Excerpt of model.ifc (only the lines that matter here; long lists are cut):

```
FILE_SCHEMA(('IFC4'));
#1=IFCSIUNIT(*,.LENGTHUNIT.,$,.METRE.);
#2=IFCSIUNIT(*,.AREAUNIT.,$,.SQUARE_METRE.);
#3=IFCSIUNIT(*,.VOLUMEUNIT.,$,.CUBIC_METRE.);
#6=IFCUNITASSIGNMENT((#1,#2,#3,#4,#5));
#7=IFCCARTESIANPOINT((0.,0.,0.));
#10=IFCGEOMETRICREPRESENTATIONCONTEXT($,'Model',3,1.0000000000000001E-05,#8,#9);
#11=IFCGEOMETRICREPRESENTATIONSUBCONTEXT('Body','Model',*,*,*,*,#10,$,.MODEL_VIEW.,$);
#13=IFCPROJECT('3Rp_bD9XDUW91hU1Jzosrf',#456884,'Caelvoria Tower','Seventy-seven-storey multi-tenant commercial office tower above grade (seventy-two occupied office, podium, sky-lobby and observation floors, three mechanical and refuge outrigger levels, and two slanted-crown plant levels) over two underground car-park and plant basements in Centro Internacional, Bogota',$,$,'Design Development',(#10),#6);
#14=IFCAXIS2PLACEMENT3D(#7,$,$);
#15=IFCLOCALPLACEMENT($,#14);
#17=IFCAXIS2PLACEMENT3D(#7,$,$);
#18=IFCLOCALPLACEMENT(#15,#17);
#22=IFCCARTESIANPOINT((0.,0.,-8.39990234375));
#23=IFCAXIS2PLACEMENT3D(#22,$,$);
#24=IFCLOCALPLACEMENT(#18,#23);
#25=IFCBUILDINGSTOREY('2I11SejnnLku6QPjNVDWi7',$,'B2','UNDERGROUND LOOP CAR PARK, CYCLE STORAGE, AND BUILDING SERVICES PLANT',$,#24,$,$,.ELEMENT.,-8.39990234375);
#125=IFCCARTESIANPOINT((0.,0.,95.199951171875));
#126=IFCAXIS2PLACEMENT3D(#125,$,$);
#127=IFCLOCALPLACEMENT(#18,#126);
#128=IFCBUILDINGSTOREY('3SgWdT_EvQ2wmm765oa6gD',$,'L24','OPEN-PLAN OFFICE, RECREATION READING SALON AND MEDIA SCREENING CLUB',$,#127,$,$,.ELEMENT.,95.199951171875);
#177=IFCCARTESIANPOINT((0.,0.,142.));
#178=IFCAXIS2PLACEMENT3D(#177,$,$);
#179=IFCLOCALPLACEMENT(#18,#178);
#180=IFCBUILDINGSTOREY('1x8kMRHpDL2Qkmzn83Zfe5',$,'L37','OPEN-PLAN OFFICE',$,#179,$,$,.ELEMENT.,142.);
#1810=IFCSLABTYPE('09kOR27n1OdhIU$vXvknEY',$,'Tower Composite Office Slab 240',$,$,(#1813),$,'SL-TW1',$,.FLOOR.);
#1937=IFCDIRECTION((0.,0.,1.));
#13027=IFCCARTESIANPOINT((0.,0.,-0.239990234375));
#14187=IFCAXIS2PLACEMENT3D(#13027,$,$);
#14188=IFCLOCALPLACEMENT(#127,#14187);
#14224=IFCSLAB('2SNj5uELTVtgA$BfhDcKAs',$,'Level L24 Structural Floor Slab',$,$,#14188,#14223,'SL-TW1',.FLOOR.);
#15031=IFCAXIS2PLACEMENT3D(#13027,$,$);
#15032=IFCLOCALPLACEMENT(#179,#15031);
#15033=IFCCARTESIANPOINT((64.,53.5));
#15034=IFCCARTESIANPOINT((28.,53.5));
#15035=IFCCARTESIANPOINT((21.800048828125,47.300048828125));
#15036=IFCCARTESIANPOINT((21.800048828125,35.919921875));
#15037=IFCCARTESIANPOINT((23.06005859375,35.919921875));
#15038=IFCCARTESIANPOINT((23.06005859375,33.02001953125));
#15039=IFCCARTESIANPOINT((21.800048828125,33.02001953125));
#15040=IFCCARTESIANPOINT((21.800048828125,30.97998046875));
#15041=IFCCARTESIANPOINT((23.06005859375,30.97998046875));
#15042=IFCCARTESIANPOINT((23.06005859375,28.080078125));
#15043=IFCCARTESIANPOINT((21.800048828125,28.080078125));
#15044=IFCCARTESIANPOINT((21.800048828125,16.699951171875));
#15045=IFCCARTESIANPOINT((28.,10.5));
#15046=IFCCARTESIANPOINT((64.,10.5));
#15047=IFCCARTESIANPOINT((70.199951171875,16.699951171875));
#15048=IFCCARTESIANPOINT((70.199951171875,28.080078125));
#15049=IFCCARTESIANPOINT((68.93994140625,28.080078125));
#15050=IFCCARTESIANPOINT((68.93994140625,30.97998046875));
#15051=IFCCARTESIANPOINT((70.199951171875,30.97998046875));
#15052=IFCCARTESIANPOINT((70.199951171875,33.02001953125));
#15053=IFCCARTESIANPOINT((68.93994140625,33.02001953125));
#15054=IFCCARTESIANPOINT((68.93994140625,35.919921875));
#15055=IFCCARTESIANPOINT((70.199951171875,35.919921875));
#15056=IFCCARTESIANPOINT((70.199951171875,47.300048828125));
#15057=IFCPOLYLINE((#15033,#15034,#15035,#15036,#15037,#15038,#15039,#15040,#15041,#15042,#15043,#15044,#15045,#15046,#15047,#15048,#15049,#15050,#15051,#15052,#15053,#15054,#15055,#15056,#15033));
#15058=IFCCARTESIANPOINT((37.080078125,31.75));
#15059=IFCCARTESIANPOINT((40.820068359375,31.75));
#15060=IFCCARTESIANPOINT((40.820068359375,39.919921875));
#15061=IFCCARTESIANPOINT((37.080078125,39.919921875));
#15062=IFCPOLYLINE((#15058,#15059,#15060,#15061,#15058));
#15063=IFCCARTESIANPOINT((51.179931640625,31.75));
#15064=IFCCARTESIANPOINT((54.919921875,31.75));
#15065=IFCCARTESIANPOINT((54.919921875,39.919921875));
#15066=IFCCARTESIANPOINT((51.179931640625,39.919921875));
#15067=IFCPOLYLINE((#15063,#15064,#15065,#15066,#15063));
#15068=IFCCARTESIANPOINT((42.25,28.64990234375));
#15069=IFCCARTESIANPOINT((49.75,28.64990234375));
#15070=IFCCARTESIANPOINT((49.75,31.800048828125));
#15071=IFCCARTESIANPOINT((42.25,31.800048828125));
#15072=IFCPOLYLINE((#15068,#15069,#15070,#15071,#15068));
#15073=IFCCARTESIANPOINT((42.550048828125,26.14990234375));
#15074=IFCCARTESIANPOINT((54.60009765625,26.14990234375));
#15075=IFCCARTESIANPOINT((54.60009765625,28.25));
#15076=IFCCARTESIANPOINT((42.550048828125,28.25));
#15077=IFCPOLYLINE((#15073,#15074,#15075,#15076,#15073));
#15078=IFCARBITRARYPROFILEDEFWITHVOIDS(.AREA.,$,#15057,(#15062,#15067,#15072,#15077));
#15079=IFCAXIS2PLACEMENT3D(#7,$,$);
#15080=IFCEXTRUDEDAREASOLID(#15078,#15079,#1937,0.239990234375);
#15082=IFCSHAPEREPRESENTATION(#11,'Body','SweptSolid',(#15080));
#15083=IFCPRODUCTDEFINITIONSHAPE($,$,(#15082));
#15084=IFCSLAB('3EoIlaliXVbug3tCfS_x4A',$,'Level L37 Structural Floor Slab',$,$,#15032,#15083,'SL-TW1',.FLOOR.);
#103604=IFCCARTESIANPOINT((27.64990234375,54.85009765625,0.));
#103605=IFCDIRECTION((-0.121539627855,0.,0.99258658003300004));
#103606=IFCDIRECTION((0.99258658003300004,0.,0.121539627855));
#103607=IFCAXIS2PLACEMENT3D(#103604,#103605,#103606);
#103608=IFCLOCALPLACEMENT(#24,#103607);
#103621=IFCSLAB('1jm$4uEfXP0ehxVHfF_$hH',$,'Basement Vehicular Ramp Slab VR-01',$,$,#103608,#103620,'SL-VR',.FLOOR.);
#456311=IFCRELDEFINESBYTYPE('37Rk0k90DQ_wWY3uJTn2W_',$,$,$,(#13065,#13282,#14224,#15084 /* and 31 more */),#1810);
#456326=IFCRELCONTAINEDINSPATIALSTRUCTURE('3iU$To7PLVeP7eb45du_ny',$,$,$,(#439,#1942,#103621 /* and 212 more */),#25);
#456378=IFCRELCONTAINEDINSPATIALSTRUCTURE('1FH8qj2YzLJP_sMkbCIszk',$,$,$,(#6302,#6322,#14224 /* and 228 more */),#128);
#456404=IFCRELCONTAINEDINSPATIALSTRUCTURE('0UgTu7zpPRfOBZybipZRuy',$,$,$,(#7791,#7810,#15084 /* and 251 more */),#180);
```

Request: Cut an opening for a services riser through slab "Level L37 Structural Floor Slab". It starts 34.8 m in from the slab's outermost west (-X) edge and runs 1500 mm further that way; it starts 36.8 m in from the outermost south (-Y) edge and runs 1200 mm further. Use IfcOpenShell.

```python
import numpy as np
import ifcopenshell
import ifcopenshell.api.feature
import ifcopenshell.api.geometry
import ifcopenshell.api.root
import ifcopenshell.geom
import ifcopenshell.util.placement
import ifcopenshell.util.representation
import ifcopenshell.util.shape
import ifcopenshell.util.unit

model = ifcopenshell.open("model.ifc")
unit_scale = ifcopenshell.util.unit.calculate_unit_scale(model)
settings = ifcopenshell.geom.settings()


def volume(element):
    """Net volume in cubic metres, openings subtracted."""
    shape = ifcopenshell.geom.create_shape(settings, element)
    return ifcopenshell.util.shape.get_volume(shape.geometry)


slab = model.by_guid("3EoIlaliXVbug3tCfS_x4A")
before = volume(slab)

# Extent in the slab's own axes, in metres. The edges named are its -X and -Y sides.
slab_shape = ifcopenshell.geom.create_shape(settings, slab)
vertices = ifcopenshell.util.shape.get_vertices(slab_shape.geometry)
x_min, y_min, bottom = vertices.min(axis=0)
top = vertices[:, 2].max()

opening = ifcopenshell.api.root.create_entity(model, ifc_class="IfcOpeningElement", name="Services riser opening", predefined_type="OPENING")
context = ifcopenshell.util.representation.get_context(model, "Model", "Body", "MODEL_VIEW")
width, depth = 1.5, 1.2
outline = [(0.0, 0.0), (width, 0.0), (width, depth), (0.0, depth), (0.0, 0.0)]
# Overshoot both faces by 50 mm so the cut is clean.
shape = ifcopenshell.api.geometry.add_slab_representation(
    model, context=context, depth=top - bottom + 0.1, polyline=outline
)
ifcopenshell.api.geometry.assign_representation(model, product=opening, representation=shape)

matrix = ifcopenshell.util.placement.get_local_placement(slab.ObjectPlacement)
matrix[:, 3] = matrix @ np.append(np.array([x_min + 34.8, y_min + 36.8, bottom - 0.05]) / unit_scale, 1.0)
ifcopenshell.api.geometry.edit_object_placement(model, product=opening, matrix=matrix, is_si=False)
ifcopenshell.api.feature.add_feature(model, feature=opening, element=slab)

after = volume(slab)

print(f"slab volume {before:.3f} -> {after:.3f} m3")

model.write("model_updated.ifc")
```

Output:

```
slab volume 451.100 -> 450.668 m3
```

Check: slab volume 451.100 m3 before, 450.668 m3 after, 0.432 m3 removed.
